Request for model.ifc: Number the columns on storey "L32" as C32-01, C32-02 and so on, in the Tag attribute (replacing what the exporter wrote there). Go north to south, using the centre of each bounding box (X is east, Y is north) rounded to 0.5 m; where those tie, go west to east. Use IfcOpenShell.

First a look at what the model holds.

```python
import ifcopenshell
import ifcopenshell.util.element
import ifcopenshell.util.placement

model = ifcopenshell.open("model.ifc")
print(model.schema)
storey = next(s for s in model.by_type("IfcBuildingStorey") if s.Name == "L32")
columns = [e for e in ifcopenshell.util.element.get_decomposition(storey) if e.is_a("IfcColumn")]
for e in sorted(columns, key=lambda e: e.id()):
    origin = ifcopenshell.util.placement.get_local_placement(e.ObjectPlacement)[:3, 3]
    print(e.id(), e.Tag, e.Name, origin.round(2) + 0.0, sep=" | ")
```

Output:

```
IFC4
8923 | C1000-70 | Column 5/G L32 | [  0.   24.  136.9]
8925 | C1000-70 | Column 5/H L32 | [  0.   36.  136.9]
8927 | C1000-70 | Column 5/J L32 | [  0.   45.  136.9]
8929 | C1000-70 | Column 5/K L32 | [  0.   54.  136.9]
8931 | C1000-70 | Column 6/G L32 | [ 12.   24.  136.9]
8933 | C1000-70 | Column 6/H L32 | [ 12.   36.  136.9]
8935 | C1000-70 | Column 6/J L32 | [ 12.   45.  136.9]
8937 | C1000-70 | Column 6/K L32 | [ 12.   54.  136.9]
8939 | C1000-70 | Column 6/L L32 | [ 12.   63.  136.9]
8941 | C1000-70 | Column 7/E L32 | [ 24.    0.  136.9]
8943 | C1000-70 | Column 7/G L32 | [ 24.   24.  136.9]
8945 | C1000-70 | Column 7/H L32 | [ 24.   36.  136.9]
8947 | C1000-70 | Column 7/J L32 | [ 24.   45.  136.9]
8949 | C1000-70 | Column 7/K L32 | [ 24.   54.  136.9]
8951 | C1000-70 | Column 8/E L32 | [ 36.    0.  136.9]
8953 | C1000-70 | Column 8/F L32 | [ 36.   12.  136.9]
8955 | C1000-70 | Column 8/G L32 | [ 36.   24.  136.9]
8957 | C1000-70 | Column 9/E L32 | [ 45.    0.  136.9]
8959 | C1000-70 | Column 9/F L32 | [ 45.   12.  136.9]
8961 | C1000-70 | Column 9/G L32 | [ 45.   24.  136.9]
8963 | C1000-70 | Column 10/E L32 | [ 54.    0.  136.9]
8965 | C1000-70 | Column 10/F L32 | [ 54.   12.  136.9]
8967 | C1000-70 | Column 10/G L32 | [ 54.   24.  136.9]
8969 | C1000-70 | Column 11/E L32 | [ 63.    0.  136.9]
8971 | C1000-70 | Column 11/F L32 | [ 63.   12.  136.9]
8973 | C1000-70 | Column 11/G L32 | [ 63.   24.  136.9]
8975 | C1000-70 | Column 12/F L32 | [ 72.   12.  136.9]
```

```python
import ifcopenshell
import ifcopenshell.geom
import ifcopenshell.util.element
import ifcopenshell.util.shape

model = ifcopenshell.open("model.ifc")
settings = ifcopenshell.geom.settings()
settings.set("use-world-coords", True)


def centre(element):
    shape = ifcopenshell.geom.create_shape(settings, element)
    return ifcopenshell.util.shape.get_bbox_centroid(shape.geometry)


storey = next(s for s in model.by_type("IfcBuildingStorey") if s.Name == "L32")
columns = [e for e in ifcopenshell.util.element.get_decomposition(storey) if e.is_a("IfcColumn")]

# Insertion points can sit at a corner or the storey origin, so sort by the geometry (in metres).
centres = {e: centre(e) for e in columns}
columns.sort(key=lambda e: (-round(centres[e][1] / 0.5), centres[e][0]))

for i, e in enumerate(columns, start=1):
    number = f"C32-{i:02d}"
    e.Tag = number
    print(e.id(), number)

model.write("model_v2.ifc")
```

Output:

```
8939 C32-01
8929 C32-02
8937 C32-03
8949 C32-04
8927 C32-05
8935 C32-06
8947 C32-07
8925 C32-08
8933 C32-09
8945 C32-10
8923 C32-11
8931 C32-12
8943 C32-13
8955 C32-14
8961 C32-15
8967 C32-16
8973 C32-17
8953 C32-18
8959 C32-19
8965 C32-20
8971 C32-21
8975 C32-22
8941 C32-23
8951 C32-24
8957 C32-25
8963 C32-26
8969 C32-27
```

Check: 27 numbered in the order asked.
